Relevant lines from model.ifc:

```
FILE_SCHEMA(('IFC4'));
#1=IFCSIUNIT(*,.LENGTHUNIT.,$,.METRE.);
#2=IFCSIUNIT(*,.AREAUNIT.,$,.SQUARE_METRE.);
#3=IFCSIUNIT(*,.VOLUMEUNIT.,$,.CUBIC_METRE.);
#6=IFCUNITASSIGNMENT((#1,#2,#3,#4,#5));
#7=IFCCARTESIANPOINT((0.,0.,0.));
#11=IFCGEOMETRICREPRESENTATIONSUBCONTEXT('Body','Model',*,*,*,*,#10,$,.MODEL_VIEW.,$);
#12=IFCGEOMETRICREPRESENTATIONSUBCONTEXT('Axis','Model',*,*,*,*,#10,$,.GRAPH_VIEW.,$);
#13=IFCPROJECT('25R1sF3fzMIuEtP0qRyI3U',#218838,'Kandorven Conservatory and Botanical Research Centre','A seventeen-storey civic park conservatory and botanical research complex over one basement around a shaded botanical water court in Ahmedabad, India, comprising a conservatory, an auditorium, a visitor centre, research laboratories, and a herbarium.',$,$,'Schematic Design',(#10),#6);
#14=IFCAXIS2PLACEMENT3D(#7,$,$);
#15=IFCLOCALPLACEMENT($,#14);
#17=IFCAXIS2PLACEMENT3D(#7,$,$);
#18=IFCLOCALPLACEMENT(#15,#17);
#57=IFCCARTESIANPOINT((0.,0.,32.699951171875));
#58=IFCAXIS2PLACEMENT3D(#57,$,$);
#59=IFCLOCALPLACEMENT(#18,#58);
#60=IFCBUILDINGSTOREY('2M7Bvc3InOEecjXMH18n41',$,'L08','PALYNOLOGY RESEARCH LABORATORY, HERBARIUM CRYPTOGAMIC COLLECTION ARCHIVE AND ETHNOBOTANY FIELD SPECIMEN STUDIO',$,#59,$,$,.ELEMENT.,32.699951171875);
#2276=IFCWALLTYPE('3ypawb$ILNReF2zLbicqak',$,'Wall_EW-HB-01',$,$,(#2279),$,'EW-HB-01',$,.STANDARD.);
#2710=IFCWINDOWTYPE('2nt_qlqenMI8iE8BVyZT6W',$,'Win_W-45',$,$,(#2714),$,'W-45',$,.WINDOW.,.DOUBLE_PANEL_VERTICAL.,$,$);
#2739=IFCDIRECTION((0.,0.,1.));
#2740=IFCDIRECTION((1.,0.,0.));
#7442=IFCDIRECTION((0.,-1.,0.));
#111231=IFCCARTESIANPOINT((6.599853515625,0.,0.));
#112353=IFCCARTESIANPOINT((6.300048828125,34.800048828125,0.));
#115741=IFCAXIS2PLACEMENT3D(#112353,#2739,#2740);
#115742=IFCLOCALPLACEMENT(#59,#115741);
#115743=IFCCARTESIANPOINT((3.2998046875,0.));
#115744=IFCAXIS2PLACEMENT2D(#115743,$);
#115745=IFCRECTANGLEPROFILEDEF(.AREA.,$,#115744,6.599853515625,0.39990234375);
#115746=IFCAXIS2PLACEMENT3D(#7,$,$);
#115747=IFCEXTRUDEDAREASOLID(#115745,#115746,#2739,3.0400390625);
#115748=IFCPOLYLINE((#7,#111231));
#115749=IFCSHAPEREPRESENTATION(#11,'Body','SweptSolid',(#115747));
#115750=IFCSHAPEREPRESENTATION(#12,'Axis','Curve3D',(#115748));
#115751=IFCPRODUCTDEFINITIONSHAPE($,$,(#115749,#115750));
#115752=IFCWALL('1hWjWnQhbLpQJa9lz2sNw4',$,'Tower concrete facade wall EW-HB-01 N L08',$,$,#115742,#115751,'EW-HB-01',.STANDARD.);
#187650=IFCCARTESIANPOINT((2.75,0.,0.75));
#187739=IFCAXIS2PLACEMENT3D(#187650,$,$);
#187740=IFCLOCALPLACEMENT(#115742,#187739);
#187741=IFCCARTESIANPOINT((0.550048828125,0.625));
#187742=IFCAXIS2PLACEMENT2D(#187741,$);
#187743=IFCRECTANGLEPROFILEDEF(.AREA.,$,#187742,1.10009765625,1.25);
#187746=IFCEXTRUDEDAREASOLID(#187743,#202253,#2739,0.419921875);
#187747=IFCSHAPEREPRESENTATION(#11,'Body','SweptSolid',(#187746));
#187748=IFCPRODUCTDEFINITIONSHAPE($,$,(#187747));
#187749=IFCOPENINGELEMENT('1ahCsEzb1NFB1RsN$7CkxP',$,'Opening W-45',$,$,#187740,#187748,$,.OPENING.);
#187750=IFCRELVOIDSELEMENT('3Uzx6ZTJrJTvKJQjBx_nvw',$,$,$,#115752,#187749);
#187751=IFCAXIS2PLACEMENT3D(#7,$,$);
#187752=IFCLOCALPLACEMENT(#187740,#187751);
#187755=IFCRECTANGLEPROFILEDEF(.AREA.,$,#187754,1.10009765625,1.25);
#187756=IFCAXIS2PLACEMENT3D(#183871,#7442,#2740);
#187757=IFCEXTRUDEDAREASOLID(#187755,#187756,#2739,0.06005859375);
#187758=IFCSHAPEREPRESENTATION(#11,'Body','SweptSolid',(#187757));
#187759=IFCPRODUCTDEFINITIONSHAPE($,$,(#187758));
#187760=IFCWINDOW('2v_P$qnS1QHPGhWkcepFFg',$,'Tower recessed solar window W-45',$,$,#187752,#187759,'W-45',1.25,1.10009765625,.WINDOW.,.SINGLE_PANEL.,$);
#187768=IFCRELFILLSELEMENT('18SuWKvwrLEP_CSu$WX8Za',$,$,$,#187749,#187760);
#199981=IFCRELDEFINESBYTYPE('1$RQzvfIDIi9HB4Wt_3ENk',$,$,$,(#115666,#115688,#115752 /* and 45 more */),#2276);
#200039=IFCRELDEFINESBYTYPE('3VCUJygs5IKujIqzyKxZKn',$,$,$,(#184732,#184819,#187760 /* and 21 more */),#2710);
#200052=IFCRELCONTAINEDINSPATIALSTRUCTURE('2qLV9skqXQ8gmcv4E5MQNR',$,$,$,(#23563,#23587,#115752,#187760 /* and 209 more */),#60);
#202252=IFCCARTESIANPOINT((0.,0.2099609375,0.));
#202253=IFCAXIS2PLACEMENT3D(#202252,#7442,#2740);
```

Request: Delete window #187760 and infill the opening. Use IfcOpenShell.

```python
import ifcopenshell
import ifcopenshell.api.feature
import ifcopenshell.api.root
import ifcopenshell.geom
import ifcopenshell.util.shape

model = ifcopenshell.open("model.ifc")
settings = ifcopenshell.geom.settings()


def volume(element):
    """Net volume in cubic metres, openings subtracted."""
    shape = ifcopenshell.geom.create_shape(settings, element)
    return ifcopenshell.util.shape.get_volume(shape.geometry)


window = model.by_guid("2v_P$qnS1QHPGhWkcepFFg")
opening = window.FillsVoids[0].RelatingOpeningElement
wall = opening.VoidsElements[0].RelatingBuildingElement
before = volume(wall)

ifcopenshell.api.root.remove_product(model, product=window)
ifcopenshell.api.feature.remove_feature(model, feature=opening)

after = volume(wall)

print(f"wall volume {before:.3f} -> {after:.3f} m3")

model.write("model_v2.ifc")
```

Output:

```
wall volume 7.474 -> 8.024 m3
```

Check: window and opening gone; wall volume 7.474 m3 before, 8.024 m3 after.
